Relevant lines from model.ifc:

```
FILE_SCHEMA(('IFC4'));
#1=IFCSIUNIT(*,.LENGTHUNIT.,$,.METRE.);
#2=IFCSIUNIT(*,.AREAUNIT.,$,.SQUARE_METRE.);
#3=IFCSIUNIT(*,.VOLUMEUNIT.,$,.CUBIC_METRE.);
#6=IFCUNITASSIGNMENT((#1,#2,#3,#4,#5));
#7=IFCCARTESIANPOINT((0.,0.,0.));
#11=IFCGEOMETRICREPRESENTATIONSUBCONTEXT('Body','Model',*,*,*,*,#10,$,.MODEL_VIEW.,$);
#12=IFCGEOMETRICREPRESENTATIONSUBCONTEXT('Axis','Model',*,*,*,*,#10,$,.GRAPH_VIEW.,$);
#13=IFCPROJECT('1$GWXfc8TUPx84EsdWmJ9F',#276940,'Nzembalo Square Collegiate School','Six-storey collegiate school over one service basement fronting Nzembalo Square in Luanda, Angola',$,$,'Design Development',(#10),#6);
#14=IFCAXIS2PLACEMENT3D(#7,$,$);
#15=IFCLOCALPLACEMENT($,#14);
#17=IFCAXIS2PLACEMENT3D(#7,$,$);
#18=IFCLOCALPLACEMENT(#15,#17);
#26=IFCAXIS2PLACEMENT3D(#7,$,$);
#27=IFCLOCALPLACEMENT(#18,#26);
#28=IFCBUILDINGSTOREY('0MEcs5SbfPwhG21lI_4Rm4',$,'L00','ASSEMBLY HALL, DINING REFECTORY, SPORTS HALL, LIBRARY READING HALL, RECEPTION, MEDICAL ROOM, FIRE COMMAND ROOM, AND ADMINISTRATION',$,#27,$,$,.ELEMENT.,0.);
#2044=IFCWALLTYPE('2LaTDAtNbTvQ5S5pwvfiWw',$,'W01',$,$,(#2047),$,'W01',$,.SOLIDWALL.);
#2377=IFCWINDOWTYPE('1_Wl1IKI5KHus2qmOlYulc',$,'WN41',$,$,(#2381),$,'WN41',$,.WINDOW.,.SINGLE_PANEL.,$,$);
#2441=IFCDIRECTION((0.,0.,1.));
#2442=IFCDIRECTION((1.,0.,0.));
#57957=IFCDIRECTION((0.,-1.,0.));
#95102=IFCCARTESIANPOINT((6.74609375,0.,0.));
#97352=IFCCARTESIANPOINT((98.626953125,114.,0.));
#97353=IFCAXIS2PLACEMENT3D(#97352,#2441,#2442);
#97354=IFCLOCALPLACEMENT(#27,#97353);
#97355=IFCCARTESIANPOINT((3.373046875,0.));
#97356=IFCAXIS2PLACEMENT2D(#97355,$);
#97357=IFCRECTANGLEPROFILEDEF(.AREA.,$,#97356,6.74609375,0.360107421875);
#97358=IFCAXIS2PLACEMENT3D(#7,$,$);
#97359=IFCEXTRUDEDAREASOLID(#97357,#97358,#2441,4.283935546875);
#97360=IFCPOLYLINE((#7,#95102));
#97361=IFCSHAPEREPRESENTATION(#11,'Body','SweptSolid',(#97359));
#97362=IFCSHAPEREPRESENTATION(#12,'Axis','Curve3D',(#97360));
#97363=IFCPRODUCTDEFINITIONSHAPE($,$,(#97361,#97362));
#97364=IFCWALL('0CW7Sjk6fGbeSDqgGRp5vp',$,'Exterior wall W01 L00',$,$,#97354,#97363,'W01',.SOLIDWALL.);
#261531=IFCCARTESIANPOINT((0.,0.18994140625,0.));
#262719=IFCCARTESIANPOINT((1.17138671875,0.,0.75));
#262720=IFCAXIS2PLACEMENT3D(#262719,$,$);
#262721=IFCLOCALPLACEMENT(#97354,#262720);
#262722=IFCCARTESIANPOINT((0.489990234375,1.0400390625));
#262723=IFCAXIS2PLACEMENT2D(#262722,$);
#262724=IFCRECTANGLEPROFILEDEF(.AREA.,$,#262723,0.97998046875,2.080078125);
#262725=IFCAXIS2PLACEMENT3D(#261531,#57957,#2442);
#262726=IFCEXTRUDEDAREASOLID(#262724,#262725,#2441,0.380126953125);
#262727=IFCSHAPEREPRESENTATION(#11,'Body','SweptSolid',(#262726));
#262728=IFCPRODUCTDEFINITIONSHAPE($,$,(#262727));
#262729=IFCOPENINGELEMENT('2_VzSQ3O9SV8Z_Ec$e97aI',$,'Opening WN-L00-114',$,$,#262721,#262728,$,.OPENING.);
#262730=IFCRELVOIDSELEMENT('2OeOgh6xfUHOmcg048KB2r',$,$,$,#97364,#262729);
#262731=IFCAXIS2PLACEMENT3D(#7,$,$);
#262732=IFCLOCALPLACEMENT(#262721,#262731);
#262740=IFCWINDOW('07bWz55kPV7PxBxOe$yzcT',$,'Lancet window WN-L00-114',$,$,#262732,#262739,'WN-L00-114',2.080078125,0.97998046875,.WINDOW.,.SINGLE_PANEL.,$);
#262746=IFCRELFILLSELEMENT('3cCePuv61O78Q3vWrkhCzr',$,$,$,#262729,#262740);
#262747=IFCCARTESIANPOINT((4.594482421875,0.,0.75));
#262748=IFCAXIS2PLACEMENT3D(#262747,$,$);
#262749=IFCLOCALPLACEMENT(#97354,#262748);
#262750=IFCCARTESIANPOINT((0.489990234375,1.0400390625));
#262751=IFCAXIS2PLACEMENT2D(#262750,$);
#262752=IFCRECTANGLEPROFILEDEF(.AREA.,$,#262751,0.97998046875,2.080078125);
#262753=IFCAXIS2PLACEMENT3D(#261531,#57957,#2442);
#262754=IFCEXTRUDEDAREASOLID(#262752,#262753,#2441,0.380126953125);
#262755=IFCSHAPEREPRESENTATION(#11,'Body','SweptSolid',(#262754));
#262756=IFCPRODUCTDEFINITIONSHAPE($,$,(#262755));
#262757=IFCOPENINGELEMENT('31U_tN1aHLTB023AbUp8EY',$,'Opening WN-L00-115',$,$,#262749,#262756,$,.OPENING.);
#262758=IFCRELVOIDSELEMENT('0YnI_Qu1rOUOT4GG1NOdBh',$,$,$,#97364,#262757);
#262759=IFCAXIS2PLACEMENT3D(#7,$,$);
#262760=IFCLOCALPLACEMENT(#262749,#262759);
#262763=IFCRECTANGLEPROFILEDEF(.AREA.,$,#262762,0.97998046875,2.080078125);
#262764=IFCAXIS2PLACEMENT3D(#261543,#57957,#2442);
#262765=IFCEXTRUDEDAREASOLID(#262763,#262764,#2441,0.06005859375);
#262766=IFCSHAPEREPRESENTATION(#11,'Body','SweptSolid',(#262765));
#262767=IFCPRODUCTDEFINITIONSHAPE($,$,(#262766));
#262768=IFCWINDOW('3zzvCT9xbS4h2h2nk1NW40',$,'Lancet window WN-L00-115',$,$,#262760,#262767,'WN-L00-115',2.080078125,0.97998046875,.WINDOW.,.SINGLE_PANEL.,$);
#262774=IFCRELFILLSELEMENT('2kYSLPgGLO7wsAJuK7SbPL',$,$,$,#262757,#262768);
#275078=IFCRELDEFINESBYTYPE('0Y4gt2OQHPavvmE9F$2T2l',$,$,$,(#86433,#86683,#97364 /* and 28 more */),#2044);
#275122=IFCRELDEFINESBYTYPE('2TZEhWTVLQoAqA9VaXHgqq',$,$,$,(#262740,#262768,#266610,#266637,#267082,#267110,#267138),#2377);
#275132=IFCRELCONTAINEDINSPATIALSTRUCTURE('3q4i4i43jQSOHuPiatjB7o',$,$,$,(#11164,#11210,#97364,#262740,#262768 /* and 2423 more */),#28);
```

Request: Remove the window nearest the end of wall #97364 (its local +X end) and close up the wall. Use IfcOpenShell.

```python
import ifcopenshell
import ifcopenshell.api.feature
import ifcopenshell.api.root
import ifcopenshell.geom
import ifcopenshell.util.shape

model = ifcopenshell.open("model.ifc")
settings = ifcopenshell.geom.settings()


def volume(element):
    """Net volume in cubic metres, openings subtracted."""
    shape = ifcopenshell.geom.create_shape(settings, element)
    return ifcopenshell.util.shape.get_volume(shape.geometry)


window = model.by_guid("3zzvCT9xbS4h2h2nk1NW40")
opening = window.FillsVoids[0].RelatingOpeningElement
wall = opening.VoidsElements[0].RelatingBuildingElement
before = volume(wall)

ifcopenshell.api.root.remove_product(model, product=window)
ifcopenshell.api.feature.remove_feature(model, feature=opening)

after = volume(wall)

print(f"wall volume {before:.3f} -> {after:.3f} m3")

model.write("model_edited.ifc")
```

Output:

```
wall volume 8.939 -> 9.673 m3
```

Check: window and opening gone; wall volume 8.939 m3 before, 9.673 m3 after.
